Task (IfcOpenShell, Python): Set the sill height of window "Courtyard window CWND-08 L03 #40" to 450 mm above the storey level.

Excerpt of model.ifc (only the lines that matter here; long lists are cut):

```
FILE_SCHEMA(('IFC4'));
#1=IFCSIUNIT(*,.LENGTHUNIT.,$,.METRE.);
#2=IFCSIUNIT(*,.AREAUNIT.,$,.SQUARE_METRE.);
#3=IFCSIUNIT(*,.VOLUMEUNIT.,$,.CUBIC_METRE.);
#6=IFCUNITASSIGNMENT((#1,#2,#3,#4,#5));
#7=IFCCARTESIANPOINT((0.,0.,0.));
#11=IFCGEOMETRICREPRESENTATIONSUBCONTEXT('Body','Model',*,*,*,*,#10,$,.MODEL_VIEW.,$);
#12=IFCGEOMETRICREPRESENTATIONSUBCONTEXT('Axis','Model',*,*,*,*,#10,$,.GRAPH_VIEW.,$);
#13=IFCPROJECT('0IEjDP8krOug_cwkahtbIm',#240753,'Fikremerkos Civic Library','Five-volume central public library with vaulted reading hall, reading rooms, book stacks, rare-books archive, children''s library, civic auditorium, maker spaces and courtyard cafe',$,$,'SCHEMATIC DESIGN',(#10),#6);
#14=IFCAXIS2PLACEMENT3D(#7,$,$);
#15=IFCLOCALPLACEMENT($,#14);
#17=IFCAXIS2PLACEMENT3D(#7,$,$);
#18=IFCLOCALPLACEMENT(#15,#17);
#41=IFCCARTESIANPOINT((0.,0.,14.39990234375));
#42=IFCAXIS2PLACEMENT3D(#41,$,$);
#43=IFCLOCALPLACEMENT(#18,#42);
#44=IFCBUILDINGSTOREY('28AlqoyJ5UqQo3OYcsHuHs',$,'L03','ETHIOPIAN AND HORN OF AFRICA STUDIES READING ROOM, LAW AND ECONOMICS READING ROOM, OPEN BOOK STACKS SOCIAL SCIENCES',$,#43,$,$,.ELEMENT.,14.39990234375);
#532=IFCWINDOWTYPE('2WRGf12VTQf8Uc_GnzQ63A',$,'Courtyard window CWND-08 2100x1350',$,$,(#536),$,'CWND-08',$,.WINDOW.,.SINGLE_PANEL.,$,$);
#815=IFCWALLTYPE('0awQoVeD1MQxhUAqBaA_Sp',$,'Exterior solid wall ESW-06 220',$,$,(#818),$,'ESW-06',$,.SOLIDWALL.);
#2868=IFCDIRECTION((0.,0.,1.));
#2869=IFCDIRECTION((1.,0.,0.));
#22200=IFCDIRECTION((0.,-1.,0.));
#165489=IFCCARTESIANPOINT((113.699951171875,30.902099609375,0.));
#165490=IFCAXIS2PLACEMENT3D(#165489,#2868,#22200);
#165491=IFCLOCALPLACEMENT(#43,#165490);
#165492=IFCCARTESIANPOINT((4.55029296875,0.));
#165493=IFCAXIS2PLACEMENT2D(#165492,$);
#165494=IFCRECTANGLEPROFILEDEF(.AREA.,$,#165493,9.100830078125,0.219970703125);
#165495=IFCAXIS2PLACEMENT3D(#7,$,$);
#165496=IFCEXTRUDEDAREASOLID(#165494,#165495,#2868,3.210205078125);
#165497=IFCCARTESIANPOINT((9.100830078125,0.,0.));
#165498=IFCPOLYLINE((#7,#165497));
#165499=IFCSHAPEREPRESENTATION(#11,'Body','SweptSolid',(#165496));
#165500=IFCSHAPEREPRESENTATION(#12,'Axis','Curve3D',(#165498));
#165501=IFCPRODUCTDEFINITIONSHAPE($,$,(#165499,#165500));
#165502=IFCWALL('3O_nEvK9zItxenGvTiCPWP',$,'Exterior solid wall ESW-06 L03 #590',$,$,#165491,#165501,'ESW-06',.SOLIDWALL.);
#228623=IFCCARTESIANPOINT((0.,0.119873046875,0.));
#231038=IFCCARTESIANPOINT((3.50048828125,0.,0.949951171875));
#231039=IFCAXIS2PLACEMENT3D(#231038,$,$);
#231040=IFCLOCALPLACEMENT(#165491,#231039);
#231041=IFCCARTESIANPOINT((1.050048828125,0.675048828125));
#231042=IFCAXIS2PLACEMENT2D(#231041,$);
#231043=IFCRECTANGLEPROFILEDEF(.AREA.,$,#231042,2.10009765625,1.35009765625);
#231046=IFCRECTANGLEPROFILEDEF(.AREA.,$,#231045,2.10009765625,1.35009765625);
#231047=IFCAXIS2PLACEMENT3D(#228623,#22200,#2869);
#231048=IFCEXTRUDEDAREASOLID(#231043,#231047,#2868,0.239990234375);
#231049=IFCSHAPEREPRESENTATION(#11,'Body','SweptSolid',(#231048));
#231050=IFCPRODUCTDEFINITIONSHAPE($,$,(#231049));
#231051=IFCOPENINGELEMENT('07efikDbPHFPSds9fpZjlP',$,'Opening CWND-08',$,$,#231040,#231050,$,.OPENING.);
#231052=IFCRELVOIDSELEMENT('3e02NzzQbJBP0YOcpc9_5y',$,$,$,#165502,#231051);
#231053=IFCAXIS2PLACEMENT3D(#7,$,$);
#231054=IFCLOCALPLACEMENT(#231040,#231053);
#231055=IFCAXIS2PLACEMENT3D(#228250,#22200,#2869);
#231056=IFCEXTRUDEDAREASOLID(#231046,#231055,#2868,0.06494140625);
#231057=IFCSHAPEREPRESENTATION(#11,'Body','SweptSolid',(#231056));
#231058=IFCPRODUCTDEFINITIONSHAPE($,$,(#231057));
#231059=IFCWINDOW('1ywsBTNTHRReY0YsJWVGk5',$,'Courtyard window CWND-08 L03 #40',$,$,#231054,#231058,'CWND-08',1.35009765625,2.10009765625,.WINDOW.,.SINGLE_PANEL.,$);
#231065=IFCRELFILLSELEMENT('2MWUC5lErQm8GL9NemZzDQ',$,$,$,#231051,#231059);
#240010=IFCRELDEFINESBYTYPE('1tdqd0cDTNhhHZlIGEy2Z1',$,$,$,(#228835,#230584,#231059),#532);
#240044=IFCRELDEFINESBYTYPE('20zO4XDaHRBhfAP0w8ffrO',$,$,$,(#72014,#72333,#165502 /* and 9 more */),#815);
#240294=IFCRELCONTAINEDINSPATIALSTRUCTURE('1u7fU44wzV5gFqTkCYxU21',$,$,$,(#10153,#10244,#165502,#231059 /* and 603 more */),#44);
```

```python
import numpy as np
import ifcopenshell
import ifcopenshell.api.geometry
import ifcopenshell.geom
import ifcopenshell.util.element
import ifcopenshell.util.placement
import ifcopenshell.util.shape
import ifcopenshell.util.unit

model = ifcopenshell.open("model.ifc")
unit_scale = ifcopenshell.util.unit.calculate_unit_scale(model)

window = model.by_id(231059)
opening = window.FillsVoids[0].RelatingOpeningElement
storey = ifcopenshell.util.element.get_container(window, ifc_class="IfcBuildingStorey")
level = ifcopenshell.util.placement.get_local_placement(storey.ObjectPlacement)[2, 3]

# The opening's origin need not be at the sill, so measure its lowest point.
shape = ifcopenshell.geom.create_shape(ifcopenshell.geom.settings(), opening)
bottom = ifcopenshell.util.shape.get_shape_bottom_elevation(shape, shape.geometry) / unit_scale
dz = level + 0.45 - bottom

shift = np.array([0.0, 0.0, dz])
# The window is placed relative to its opening, so it follows when the opening moves.
matrix = ifcopenshell.util.placement.get_local_placement(opening.ObjectPlacement)
matrix[:3, 3] += shift
ifcopenshell.api.geometry.edit_object_placement(
    model, product=opening, matrix=matrix, is_si=False, should_transform_children=True
)

print(f"moved by {dz * unit_scale:+.3f} m")

model.write("model_v2.ifc")
```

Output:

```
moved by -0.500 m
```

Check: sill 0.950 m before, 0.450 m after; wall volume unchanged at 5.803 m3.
